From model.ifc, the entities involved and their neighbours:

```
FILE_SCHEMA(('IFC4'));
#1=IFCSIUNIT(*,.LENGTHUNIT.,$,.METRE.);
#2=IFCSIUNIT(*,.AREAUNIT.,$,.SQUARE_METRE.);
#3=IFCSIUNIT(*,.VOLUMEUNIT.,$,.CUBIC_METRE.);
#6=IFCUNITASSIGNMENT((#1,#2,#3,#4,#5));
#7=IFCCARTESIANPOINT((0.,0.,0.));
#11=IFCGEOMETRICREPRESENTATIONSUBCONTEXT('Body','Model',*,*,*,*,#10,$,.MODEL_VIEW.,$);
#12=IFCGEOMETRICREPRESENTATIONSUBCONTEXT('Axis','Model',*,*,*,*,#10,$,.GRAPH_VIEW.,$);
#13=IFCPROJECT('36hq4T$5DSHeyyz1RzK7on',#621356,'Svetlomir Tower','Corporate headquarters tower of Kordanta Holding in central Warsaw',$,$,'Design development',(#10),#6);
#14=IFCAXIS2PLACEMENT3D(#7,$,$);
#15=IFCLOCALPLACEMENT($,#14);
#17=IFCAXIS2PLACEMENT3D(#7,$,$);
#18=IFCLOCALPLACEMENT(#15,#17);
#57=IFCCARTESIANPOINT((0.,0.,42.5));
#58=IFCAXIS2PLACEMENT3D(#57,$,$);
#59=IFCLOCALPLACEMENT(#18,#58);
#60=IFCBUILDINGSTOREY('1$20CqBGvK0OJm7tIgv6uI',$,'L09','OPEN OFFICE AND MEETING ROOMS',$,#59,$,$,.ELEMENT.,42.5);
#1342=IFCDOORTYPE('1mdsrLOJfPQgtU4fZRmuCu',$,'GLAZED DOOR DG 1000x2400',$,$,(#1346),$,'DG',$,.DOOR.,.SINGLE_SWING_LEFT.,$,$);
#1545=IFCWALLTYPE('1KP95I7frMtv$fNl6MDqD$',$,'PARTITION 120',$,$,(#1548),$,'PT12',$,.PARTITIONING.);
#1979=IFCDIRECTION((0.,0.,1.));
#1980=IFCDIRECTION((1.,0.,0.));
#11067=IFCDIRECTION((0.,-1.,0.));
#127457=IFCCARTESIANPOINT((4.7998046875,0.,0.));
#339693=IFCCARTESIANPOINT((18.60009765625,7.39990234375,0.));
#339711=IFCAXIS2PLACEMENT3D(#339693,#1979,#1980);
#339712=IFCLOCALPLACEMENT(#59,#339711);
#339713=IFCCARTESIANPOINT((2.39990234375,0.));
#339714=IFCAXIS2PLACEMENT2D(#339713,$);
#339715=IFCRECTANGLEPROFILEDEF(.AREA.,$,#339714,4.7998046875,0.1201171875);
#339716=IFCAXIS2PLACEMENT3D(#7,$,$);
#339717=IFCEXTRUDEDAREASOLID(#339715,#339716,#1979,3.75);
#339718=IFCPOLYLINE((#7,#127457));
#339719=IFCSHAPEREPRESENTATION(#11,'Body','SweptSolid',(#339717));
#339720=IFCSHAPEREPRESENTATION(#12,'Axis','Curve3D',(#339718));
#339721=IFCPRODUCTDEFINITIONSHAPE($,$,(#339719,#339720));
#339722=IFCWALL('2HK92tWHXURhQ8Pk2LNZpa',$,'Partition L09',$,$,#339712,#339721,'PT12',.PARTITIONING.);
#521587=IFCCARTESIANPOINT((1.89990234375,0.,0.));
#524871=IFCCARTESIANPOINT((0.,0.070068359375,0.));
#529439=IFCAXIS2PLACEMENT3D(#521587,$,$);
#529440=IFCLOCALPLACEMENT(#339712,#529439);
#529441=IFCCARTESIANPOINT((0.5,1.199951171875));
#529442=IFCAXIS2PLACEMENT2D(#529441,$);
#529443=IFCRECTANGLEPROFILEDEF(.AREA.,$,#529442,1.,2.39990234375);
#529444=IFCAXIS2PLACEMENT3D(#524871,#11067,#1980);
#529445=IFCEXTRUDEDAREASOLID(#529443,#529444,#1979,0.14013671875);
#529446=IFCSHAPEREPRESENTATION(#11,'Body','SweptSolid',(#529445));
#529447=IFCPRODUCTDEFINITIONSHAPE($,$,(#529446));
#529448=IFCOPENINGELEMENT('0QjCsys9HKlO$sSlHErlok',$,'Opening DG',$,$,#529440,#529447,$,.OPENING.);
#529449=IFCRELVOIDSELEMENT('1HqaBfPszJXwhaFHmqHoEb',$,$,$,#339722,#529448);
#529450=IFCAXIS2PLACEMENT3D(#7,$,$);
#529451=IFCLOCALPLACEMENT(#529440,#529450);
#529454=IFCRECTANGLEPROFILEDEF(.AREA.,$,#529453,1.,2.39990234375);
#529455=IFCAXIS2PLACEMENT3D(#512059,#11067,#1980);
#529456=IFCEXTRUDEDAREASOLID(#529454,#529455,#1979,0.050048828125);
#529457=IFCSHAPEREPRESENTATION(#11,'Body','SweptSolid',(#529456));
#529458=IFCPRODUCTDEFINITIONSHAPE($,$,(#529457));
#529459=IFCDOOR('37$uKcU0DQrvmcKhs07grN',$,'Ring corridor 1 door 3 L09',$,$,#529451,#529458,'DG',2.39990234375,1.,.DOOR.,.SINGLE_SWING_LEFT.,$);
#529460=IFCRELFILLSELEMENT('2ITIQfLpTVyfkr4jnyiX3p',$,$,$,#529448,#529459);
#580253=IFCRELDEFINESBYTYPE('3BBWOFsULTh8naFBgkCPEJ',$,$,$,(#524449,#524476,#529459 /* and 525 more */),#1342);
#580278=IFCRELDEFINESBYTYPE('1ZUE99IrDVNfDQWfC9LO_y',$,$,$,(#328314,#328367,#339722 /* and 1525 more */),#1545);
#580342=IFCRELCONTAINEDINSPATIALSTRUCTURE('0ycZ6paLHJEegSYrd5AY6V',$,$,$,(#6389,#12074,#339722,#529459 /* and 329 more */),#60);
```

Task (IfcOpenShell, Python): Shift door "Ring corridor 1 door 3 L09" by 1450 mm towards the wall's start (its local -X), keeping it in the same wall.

```python
import ifcopenshell
import ifcopenshell.api.geometry
import ifcopenshell.util.placement
import ifcopenshell.util.unit

model = ifcopenshell.open("model.ifc")
unit_scale = ifcopenshell.util.unit.calculate_unit_scale(model)

door = model.by_guid("37$uKcU0DQrvmcKhs07grN")
opening = door.FillsVoids[0].RelatingOpeningElement
wall = opening.VoidsElements[0].RelatingBuildingElement

wall_matrix = ifcopenshell.util.placement.get_local_placement(wall.ObjectPlacement)
shift = wall_matrix[:3, 0] * -1.45 / unit_scale
before = ifcopenshell.util.placement.get_local_placement(door.ObjectPlacement)[:3, 3].copy()

# The door is placed relative to its opening, so it follows when the opening moves.
matrix = ifcopenshell.util.placement.get_local_placement(opening.ObjectPlacement)
matrix[:3, 3] += shift
ifcopenshell.api.geometry.edit_object_placement(
    model, product=opening, matrix=matrix, is_si=False, should_transform_children=True
)

after = ifcopenshell.util.placement.get_local_placement(door.ObjectPlacement)[:3, 3]
print("door moved by", (after - before).round(3) + 0.0)

model.write("model_edited.ifc")
```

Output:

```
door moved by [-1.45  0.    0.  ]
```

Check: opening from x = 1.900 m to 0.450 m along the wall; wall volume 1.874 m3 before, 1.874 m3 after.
